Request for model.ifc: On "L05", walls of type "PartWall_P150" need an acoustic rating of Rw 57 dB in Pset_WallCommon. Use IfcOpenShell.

First a look at what the model holds.

```python
import ifcopenshell
import ifcopenshell.util.element

model = ifcopenshell.open("model.ifc")
print(model.schema)
storey = next(s for s in model.by_type("IfcBuildingStorey") if s.Name == "L05")
walls = [e for e in ifcopenshell.util.element.get_decomposition(storey) if e.is_a("IfcWall")]
seen = {}
for e in walls:
    element_type = ifcopenshell.util.element.get_type(e)
    key = (element_type.Name if element_type != e and element_type else None, ifcopenshell.util.element.get_pset(e, "Pset_WallCommon", "AcousticRating"))
    seen[key] = seen.get(key, 0) + 1
for (name, value), count in sorted(seen.items(), key=str):
    print(count, "x", name, "|", value)
```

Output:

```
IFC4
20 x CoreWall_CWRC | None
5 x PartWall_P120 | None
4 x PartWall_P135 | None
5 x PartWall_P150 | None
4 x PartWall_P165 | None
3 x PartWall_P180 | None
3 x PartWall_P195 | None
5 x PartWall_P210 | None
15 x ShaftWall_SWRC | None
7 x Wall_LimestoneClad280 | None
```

```python
import ifcopenshell
import ifcopenshell.api.pset
import ifcopenshell.util.element

model = ifcopenshell.open("model.ifc")

storey = next(s for s in model.by_type("IfcBuildingStorey") if s.Name == "L05")
walls = [e for e in ifcopenshell.util.element.get_decomposition(storey) if e.is_a("IfcWall")]

count = 0
for e in walls:
    element_type = ifcopenshell.util.element.get_type(e)
    if element_type in (None, e) or element_type.Name != "PartWall_P150":
        continue
    # add_pset returns the element's existing set when there is one.
    pset = ifcopenshell.api.pset.add_pset(model, product=e, name="Pset_WallCommon")
    ifcopenshell.api.pset.edit_pset(model, pset=pset, properties={"AcousticRating": "Rw 57 dB"})
    count += 1

print(count, "walls updated")

model.write("model-out.ifc")
```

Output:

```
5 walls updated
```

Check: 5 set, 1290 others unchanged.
